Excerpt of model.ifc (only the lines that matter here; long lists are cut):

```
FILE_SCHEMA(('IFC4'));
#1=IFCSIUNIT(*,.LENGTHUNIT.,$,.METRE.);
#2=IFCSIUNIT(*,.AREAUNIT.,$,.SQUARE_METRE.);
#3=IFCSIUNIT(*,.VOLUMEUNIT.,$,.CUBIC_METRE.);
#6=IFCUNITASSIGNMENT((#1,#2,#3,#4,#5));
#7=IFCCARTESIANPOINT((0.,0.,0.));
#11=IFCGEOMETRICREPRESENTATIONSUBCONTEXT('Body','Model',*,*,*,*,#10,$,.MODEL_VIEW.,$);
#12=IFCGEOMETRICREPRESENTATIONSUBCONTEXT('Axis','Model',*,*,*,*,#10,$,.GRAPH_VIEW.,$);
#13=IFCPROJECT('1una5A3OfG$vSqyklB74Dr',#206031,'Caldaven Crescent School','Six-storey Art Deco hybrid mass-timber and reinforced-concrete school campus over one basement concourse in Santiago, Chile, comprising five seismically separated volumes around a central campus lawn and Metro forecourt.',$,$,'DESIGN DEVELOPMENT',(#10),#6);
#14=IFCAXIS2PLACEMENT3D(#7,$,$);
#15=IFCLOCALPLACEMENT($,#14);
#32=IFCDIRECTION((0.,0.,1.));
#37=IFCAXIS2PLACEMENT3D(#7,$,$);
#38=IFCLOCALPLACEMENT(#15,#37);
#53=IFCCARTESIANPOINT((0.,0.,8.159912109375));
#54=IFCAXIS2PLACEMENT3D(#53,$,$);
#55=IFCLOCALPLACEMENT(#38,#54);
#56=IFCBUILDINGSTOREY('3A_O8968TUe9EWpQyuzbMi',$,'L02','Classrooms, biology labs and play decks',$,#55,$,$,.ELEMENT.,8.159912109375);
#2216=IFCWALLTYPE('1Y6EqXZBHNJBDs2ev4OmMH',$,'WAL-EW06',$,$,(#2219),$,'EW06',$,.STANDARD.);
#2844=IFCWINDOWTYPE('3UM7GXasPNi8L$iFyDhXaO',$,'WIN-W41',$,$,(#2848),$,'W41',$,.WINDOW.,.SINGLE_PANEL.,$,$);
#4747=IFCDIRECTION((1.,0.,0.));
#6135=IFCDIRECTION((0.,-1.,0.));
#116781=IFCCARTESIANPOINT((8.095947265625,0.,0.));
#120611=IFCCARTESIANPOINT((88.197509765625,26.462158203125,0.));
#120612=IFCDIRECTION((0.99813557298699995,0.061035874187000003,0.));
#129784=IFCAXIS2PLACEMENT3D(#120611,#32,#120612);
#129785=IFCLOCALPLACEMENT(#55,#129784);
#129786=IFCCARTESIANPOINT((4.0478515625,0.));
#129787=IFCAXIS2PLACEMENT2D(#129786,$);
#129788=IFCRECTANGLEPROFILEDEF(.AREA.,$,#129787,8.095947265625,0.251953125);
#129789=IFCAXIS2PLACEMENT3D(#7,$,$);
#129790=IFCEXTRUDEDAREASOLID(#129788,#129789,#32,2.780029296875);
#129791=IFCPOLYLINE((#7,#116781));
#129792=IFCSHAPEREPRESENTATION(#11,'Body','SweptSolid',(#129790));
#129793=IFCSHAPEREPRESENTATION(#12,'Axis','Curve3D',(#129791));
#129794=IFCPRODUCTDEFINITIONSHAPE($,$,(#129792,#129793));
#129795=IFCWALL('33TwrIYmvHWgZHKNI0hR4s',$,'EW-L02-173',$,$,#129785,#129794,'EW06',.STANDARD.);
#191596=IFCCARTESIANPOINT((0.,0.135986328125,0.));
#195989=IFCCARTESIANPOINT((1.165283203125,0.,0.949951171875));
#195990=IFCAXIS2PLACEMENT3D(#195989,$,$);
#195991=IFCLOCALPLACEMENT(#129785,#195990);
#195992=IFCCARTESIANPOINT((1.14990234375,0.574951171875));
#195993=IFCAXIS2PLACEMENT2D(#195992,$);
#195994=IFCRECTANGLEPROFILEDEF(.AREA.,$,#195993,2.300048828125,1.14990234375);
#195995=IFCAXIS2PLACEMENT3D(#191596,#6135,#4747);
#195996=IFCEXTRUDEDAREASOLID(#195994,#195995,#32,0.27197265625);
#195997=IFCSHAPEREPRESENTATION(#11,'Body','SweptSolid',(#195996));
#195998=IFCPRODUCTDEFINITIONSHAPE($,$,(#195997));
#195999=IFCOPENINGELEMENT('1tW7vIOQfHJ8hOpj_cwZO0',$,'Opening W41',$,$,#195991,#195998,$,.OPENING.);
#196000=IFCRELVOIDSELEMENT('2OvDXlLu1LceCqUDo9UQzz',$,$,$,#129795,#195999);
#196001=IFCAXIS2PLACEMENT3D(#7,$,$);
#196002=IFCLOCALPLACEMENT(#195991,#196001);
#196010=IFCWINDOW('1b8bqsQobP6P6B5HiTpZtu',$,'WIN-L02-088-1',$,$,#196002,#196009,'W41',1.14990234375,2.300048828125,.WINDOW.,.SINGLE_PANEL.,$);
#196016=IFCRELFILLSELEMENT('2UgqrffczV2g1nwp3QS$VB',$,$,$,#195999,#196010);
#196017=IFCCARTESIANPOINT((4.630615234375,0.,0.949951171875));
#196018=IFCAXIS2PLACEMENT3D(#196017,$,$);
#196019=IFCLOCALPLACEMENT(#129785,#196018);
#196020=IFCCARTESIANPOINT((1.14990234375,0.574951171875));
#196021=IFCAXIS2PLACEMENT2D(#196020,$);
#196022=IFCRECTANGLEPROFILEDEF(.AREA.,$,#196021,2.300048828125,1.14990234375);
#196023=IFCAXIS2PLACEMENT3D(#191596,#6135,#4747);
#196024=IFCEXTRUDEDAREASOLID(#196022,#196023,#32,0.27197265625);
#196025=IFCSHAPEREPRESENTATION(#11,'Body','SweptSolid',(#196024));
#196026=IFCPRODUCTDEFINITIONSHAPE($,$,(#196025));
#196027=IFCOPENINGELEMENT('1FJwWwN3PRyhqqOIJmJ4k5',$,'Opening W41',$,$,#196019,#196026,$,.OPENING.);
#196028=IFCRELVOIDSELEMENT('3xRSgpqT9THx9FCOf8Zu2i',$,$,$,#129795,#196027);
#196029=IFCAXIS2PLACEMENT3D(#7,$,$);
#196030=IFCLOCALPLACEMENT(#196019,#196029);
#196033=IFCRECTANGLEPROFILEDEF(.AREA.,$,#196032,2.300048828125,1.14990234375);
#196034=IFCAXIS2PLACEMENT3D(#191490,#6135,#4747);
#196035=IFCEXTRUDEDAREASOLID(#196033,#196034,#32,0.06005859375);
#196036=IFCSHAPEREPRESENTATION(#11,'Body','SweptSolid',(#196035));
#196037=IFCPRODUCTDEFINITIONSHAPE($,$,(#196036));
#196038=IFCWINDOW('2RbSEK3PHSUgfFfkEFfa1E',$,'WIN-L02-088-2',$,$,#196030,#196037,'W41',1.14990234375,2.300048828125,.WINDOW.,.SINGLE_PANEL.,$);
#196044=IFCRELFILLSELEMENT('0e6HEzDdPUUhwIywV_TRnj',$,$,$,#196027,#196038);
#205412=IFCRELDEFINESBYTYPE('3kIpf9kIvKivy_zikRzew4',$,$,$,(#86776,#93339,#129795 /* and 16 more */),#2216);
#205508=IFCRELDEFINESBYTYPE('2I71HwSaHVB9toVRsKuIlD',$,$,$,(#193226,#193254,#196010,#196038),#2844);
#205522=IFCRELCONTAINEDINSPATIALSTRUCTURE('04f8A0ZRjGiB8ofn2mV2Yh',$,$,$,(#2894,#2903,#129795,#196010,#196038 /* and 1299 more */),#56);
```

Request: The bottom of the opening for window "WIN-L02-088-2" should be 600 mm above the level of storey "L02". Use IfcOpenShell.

```python
import numpy as np
import ifcopenshell
import ifcopenshell.api.geometry
import ifcopenshell.geom
import ifcopenshell.util.element
import ifcopenshell.util.placement
import ifcopenshell.util.shape
import ifcopenshell.util.unit

model = ifcopenshell.open("model.ifc")
unit_scale = ifcopenshell.util.unit.calculate_unit_scale(model)

window = model.by_id(196038)
opening = window.FillsVoids[0].RelatingOpeningElement
storey = ifcopenshell.util.element.get_container(window, ifc_class="IfcBuildingStorey")
level = ifcopenshell.util.placement.get_local_placement(storey.ObjectPlacement)[2, 3]

# The opening's origin need not be at the sill, so measure its lowest point.
shape = ifcopenshell.geom.create_shape(ifcopenshell.geom.settings(), opening)
bottom = ifcopenshell.util.shape.get_shape_bottom_elevation(shape, shape.geometry) / unit_scale
dz = level + 0.6 - bottom

shift = np.array([0.0, 0.0, dz])
# The window is placed relative to its opening, so it follows when the opening moves.
matrix = ifcopenshell.util.placement.get_local_placement(opening.ObjectPlacement)
matrix[:3, 3] += shift
ifcopenshell.api.geometry.edit_object_placement(
    model, product=opening, matrix=matrix, is_si=False, should_transform_children=True
)

print(f"moved by {dz * unit_scale:+.3f} m")

model.write("model_rev.ifc")
```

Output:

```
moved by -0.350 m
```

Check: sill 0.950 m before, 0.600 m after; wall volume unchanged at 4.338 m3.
